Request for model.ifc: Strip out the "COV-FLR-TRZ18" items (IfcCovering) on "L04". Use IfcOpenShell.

First a look at what the model holds.

```python
import ifcopenshell
import ifcopenshell.util.element

model = ifcopenshell.open("model.ifc")
print(model.schema)
storey = next(s for s in model.by_type("IfcBuildingStorey") if s.Name == "L04")
coverings = [e for e in ifcopenshell.util.element.get_decomposition(storey) if e.is_a("IfcCovering")]
seen = {}
for e in coverings:
    element_type = ifcopenshell.util.element.get_type(e)
    name = element_type.Name if element_type not in (None, e) else None
    seen[name] = seen.get(name, 0) + 1
for name, count in sorted(seen.items(), key=str):
    print(count, "x", name)
```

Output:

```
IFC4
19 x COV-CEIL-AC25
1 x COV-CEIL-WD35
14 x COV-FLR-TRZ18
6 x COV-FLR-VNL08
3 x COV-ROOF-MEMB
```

```python
import ifcopenshell
import ifcopenshell.api.root
import ifcopenshell.util.element

model = ifcopenshell.open("model.ifc")

storey = next(s for s in model.by_type("IfcBuildingStorey") if s.Name == "L04")
coverings = [e for e in ifcopenshell.util.element.get_decomposition(storey) if e.is_a("IfcCovering")]
targets = [e for e in coverings if (t := ifcopenshell.util.element.get_type(e)) not in (None, e) and t.Name == "COV-FLR-TRZ18"]

for e in targets:
    ifcopenshell.api.root.remove_product(model, product=e)
print(len(targets), "removed")

model.write("model_updated.ifc")
```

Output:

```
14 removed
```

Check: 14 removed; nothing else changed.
